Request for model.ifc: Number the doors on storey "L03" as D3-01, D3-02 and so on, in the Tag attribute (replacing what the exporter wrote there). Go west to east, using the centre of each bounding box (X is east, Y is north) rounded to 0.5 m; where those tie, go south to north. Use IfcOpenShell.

First a look at what the model holds.

```python
import ifcopenshell
import ifcopenshell.util.element
import ifcopenshell.util.placement

model = ifcopenshell.open("model.ifc")
print(model.schema)
storey = next(s for s in model.by_type("IfcBuildingStorey") if s.Name == "L03")
doors = [e for e in ifcopenshell.util.element.get_decomposition(storey) if e.is_a("IfcDoor")]
for e in sorted(doors, key=lambda e: e.id()):
    origin = ifcopenshell.util.placement.get_local_placement(e.ObjectPlacement)[:3, 3]
    print(e.id(), e.Tag, e.Name, origin.round(2) + 0.0, sep=" | ")
```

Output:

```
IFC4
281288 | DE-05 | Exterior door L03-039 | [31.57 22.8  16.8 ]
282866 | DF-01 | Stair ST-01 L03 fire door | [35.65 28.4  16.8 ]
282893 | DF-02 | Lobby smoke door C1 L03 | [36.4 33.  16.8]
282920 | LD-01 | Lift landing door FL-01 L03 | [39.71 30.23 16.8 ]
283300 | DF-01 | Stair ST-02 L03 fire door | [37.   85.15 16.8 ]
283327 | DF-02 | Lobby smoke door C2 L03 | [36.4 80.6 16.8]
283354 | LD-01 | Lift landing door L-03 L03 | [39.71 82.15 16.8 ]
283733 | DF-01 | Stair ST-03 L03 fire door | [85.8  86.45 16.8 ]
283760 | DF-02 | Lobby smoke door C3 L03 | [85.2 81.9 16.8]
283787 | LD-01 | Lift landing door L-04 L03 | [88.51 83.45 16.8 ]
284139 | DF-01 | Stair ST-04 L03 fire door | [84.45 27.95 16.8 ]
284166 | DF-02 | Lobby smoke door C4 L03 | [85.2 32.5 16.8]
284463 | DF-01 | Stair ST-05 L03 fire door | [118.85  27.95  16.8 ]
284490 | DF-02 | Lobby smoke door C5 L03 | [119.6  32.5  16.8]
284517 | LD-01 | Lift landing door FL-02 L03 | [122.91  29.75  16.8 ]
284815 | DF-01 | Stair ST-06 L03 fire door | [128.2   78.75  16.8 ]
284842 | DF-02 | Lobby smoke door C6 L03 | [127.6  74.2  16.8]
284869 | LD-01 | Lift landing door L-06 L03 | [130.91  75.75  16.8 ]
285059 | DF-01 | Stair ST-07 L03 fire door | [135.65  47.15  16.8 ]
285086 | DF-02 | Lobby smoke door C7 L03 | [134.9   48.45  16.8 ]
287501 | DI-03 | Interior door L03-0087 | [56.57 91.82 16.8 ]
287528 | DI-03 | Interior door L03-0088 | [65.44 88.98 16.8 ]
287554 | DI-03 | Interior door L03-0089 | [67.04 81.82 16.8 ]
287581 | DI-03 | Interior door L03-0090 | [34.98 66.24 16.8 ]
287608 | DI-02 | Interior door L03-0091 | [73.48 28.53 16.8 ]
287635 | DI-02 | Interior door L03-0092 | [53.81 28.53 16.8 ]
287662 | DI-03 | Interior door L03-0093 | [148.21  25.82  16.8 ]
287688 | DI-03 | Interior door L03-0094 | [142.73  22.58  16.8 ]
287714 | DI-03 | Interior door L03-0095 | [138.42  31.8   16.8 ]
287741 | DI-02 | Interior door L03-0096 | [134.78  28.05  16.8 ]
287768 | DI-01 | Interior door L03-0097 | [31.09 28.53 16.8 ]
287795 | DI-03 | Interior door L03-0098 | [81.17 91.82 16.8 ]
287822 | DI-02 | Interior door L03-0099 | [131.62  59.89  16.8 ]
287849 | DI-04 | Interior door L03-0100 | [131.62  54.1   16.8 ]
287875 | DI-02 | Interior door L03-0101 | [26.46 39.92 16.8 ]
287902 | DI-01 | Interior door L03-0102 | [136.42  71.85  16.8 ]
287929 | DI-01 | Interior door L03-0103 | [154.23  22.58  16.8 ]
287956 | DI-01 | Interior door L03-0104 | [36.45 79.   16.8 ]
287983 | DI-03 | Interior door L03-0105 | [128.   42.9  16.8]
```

```python
import ifcopenshell
import ifcopenshell.geom
import ifcopenshell.util.element
import ifcopenshell.util.shape

model = ifcopenshell.open("model.ifc")
settings = ifcopenshell.geom.settings()
settings.set("use-world-coords", True)


def centre(element):
    shape = ifcopenshell.geom.create_shape(settings, element)
    return ifcopenshell.util.shape.get_bbox_centroid(shape.geometry)


storey = next(s for s in model.by_type("IfcBuildingStorey") if s.Name == "L03")
doors = [e for e in ifcopenshell.util.element.get_decomposition(storey) if e.is_a("IfcDoor")]

# Insertion points can sit at a corner or the storey origin, so sort by the geometry (in metres).
centres = {e: centre(e) for e in doors}
doors.sort(key=lambda e: (round(centres[e][0] / 0.5), centres[e][1]))

for i, e in enumerate(doors, start=1):
    number = f"D3-{i:02d}"
    e.Tag = number
    print(e.id(), number)

model.write("model_rev.ifc")
```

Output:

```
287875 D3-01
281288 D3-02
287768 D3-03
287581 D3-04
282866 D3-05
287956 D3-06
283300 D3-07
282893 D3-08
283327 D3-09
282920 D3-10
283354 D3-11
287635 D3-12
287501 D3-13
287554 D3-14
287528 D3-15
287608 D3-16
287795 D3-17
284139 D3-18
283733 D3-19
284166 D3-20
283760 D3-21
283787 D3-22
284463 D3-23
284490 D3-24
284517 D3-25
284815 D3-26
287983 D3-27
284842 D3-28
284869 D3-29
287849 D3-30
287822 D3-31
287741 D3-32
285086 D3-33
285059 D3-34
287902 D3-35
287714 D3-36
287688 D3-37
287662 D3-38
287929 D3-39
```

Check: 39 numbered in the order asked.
